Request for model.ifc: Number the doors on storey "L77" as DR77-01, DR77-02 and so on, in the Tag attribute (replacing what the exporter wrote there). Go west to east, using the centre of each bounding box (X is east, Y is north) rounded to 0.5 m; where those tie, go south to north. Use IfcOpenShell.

First a look at what the model holds.

```python
import ifcopenshell
import ifcopenshell.util.element
import ifcopenshell.util.placement

model = ifcopenshell.open("model.ifc")
print(model.schema)
storey = next(s for s in model.by_type("IfcBuildingStorey") if s.Name == "L77")
doors = [e for e in ifcopenshell.util.element.get_decomposition(storey) if e.is_a("IfcDoor")]
for e in sorted(doors, key=lambda e: e.id()):
    origin = ifcopenshell.util.placement.get_local_placement(e.ObjectPlacement)[:3, 3]
    print(e.id(), e.Tag, e.Name, origin.round(2) + 0.0, sep=" | ")
```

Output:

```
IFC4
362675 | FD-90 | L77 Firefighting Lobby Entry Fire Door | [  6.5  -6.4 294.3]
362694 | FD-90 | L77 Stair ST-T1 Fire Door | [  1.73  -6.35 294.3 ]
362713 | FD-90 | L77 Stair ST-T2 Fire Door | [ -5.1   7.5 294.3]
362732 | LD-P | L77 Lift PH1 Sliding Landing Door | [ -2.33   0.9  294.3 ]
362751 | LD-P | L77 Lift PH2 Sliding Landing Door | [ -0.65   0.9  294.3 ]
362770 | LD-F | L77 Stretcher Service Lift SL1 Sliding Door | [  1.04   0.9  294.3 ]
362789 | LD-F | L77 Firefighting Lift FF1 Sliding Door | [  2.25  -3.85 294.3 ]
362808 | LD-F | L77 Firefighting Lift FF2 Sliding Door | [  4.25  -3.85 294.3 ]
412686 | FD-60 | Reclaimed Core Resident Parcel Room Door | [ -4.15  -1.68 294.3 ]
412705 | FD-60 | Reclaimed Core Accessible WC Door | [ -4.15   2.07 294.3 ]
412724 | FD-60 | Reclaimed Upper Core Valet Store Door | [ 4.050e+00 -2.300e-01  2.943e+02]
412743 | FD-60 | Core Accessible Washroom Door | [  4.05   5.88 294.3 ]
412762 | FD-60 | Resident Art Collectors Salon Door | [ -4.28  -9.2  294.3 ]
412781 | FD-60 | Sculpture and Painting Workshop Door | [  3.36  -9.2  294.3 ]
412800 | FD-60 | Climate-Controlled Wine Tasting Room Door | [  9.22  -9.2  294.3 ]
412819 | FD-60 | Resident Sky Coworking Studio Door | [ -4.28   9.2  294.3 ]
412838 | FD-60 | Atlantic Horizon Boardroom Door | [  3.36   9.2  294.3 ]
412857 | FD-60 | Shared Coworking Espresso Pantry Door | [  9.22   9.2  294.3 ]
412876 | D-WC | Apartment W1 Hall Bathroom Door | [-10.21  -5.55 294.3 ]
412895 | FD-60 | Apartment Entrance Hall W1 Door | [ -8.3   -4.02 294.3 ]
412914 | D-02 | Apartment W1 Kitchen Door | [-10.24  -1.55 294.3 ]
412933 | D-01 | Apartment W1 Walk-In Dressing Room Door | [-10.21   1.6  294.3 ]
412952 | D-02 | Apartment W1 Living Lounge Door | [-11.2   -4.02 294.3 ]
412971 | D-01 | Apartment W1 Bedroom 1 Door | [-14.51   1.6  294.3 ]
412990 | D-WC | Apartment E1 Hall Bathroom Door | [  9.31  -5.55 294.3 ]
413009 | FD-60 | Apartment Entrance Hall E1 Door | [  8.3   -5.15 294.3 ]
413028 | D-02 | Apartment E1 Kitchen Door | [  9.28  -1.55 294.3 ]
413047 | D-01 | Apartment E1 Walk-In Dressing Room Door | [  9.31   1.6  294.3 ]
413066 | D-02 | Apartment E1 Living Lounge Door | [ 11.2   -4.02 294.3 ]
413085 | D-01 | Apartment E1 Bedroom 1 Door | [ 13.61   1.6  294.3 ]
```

```python
import ifcopenshell
import ifcopenshell.geom
import ifcopenshell.util.element
import ifcopenshell.util.shape

model = ifcopenshell.open("model.ifc")
settings = ifcopenshell.geom.settings()
settings.set("use-world-coords", True)


def centre(element):
    shape = ifcopenshell.geom.create_shape(settings, element)
    return ifcopenshell.util.shape.get_bbox_centroid(shape.geometry)


storey = next(s for s in model.by_type("IfcBuildingStorey") if s.Name == "L77")
doors = [e for e in ifcopenshell.util.element.get_decomposition(storey) if e.is_a("IfcDoor")]

# Insertion points can sit at a corner or the storey origin, so sort by the geometry (in metres).
centres = {e: centre(e) for e in doors}
doors.sort(key=lambda e: (round(centres[e][0] / 0.5), centres[e][1]))

for i, e in enumerate(doors, start=1):
    number = f"DR77-{i:02d}"
    e.Tag = number
    print(e.id(), number)

model.write("model_updated.ifc")
```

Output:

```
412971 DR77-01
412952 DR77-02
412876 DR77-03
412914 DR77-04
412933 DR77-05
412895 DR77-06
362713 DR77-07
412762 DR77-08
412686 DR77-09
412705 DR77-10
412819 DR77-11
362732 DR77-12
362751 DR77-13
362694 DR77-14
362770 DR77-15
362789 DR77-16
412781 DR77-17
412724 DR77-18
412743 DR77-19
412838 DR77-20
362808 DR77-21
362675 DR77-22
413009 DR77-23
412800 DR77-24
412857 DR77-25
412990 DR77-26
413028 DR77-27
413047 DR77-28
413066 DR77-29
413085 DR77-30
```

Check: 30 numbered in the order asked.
